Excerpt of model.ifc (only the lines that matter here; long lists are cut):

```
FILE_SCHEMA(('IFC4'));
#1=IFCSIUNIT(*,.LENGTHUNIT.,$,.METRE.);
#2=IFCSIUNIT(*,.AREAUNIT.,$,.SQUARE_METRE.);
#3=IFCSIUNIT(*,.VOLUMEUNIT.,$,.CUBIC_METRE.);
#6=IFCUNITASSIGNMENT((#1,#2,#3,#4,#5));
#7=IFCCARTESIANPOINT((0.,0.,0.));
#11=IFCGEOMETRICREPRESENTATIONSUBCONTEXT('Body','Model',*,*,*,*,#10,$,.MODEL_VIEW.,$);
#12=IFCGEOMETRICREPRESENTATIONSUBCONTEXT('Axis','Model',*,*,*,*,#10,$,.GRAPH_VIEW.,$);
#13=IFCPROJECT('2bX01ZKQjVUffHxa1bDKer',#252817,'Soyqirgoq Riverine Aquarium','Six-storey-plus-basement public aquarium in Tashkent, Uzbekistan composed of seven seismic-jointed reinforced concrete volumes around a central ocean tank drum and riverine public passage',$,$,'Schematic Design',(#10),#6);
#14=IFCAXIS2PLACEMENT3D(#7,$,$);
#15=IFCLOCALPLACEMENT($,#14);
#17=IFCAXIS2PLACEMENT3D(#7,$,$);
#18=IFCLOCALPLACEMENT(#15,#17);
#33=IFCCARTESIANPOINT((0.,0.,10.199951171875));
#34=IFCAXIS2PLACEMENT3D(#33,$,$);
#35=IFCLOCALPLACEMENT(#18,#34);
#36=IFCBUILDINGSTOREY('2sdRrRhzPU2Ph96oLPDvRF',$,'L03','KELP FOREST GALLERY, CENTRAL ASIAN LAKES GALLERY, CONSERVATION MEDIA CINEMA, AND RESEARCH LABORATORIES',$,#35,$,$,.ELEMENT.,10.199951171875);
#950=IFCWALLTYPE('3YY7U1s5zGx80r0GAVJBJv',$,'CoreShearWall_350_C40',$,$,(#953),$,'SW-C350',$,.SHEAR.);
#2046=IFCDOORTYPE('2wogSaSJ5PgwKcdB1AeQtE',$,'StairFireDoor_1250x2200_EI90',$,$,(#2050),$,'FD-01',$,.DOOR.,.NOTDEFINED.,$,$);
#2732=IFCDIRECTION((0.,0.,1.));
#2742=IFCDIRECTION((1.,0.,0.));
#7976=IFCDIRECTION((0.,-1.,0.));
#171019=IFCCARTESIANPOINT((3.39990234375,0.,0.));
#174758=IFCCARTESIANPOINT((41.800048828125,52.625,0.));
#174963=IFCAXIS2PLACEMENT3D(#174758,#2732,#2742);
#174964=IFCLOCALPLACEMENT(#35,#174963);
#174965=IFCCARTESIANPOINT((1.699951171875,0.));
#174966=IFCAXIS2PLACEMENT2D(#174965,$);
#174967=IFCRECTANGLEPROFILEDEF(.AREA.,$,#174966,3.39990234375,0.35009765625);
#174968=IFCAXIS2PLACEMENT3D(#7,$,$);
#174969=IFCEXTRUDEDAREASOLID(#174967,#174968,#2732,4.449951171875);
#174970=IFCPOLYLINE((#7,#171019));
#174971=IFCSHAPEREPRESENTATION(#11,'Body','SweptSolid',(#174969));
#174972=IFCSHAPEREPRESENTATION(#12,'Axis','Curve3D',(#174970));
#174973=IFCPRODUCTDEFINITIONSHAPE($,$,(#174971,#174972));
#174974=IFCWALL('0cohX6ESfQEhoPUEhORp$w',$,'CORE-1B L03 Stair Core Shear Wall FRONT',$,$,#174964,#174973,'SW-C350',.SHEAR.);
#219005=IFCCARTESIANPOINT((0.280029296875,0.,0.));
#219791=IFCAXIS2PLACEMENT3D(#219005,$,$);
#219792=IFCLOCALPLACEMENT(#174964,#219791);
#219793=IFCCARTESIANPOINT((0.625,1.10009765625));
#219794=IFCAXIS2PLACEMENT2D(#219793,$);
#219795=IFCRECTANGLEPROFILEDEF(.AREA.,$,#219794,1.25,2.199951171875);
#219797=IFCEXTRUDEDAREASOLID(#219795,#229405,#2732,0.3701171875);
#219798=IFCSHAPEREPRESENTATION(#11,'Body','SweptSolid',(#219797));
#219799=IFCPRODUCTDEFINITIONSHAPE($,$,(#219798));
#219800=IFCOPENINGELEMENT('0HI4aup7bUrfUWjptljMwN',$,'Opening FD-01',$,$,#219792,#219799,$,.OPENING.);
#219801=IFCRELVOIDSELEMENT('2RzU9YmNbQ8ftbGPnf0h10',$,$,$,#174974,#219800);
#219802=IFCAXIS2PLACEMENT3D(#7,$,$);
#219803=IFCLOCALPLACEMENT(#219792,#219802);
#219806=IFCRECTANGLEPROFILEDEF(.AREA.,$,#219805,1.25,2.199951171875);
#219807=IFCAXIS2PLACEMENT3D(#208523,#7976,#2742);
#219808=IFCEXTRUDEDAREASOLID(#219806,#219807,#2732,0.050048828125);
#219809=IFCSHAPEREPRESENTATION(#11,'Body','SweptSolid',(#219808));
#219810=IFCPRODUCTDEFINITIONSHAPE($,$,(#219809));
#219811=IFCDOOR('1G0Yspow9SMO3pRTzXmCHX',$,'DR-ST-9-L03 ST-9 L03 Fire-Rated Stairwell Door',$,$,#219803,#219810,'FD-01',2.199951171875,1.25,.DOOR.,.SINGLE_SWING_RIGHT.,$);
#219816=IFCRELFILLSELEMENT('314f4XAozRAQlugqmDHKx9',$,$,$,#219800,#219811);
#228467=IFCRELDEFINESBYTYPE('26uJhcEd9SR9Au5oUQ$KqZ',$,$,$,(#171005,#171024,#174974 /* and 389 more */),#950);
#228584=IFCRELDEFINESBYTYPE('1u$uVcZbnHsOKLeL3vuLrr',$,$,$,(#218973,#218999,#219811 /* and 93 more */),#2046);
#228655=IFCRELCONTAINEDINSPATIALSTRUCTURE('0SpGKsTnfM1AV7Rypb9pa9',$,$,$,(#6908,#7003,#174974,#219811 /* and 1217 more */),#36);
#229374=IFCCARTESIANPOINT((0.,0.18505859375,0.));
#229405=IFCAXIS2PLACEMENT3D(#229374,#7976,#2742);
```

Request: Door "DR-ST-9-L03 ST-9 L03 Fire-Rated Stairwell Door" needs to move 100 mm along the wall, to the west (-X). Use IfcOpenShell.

```python
import ifcopenshell
import ifcopenshell.api.geometry
import ifcopenshell.util.placement
import ifcopenshell.util.unit

model = ifcopenshell.open("model.ifc")
unit_scale = ifcopenshell.util.unit.calculate_unit_scale(model)

door = model.by_guid("1G0Yspow9SMO3pRTzXmCHX")
opening = door.FillsVoids[0].RelatingOpeningElement
wall = opening.VoidsElements[0].RelatingBuildingElement

wall_matrix = ifcopenshell.util.placement.get_local_placement(wall.ObjectPlacement)
shift = wall_matrix[:3, 0] * -0.1 / unit_scale
before = ifcopenshell.util.placement.get_local_placement(door.ObjectPlacement)[:3, 3].copy()

# The door is placed relative to its opening, so it follows when the opening moves.
matrix = ifcopenshell.util.placement.get_local_placement(opening.ObjectPlacement)
matrix[:3, 3] += shift
ifcopenshell.api.geometry.edit_object_placement(
    model, product=opening, matrix=matrix, is_si=False, should_transform_children=True
)

after = ifcopenshell.util.placement.get_local_placement(door.ObjectPlacement)[:3, 3]
print("door moved by", (after - before).round(3) + 0.0)

model.write("model-out.ifc")
```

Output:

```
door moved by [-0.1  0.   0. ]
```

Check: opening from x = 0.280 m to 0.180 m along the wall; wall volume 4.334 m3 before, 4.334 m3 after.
